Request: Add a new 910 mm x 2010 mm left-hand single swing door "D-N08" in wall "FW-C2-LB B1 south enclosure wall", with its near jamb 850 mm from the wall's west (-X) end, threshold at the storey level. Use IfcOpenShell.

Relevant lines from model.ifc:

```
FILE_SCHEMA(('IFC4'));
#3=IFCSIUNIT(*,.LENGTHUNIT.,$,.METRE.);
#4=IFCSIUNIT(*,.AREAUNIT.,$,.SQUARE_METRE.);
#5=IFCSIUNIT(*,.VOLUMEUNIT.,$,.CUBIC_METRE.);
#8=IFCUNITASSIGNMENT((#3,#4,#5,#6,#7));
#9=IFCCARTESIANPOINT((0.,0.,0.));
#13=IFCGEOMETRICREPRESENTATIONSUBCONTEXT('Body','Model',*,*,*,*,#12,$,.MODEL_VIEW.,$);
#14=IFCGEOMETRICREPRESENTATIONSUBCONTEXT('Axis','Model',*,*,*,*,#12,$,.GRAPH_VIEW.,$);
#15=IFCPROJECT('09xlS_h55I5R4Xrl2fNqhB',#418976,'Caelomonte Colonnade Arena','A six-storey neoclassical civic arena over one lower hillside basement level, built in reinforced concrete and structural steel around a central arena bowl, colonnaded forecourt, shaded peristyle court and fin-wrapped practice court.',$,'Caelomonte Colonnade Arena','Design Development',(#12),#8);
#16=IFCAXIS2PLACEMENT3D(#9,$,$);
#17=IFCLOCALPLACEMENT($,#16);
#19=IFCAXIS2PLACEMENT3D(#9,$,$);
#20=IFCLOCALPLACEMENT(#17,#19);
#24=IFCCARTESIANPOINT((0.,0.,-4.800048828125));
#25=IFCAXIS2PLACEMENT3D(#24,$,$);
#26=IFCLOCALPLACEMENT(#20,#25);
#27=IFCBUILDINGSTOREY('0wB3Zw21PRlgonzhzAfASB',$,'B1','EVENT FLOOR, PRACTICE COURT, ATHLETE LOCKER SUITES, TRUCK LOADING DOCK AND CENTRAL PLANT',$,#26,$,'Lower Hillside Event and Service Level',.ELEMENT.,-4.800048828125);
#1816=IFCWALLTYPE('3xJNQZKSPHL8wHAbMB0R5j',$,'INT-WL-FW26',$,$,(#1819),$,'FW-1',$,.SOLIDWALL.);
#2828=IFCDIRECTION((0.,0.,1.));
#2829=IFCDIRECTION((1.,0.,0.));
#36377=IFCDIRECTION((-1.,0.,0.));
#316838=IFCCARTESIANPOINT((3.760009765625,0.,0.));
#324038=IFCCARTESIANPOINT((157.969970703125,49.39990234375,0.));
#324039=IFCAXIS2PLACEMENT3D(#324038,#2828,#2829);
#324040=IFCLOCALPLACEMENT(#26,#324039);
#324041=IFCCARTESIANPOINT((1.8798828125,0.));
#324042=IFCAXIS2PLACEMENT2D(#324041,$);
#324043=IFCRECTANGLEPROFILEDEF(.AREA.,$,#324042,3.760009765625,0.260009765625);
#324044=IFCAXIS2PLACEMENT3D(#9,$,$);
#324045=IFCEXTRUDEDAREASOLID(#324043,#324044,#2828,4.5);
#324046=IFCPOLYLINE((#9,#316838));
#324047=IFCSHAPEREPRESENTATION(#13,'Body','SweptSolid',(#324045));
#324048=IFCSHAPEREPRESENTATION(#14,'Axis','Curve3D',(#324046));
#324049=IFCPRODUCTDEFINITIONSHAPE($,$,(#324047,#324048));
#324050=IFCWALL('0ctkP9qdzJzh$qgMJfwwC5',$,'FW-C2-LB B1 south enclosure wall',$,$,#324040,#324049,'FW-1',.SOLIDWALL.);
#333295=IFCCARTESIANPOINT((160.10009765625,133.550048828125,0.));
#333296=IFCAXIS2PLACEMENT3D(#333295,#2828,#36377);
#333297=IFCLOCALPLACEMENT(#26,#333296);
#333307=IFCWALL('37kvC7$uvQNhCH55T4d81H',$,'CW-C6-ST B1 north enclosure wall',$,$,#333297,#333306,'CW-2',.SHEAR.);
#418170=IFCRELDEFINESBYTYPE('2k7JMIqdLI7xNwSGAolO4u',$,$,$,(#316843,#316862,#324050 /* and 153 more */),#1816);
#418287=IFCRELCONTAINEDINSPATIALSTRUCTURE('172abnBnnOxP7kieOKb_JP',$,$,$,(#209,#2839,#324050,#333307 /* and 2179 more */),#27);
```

```python
import numpy as np
import ifcopenshell
import ifcopenshell.api.feature
import ifcopenshell.api.geometry
import ifcopenshell.api.root
import ifcopenshell.api.spatial
import ifcopenshell.geom
import ifcopenshell.util.element
import ifcopenshell.util.placement
import ifcopenshell.util.representation
import ifcopenshell.util.shape
import ifcopenshell.util.unit

model = ifcopenshell.open("model.ifc")
unit_scale = ifcopenshell.util.unit.calculate_unit_scale(model)
settings = ifcopenshell.geom.settings()


def volume(element):
    """Net volume in cubic metres, openings subtracted."""
    shape = ifcopenshell.geom.create_shape(settings, element)
    return ifcopenshell.util.shape.get_volume(shape.geometry)


wall = model.by_id(324050)
storey = ifcopenshell.util.element.get_container(wall, ifc_class="IfcBuildingStorey")
context = ifcopenshell.util.representation.get_context(model, "Model", "Body", "MODEL_VIEW")
before = volume(wall)

width, height, from_end, sill = 0.91, 2.01, 0.85, 0.0  # metres

# The wall runs along its own X axis, and the end named is its -X end.
wall_shape = ifcopenshell.geom.create_shape(settings, wall)
x, y, z = ifcopenshell.util.shape.get_vertices(wall_shape.geometry).T
start = x.min() + from_end
face, thickness = float(y.min()), float(y.max() - y.min())
wall_matrix = ifcopenshell.util.placement.get_local_placement(wall.ObjectPlacement)
level = ifcopenshell.util.placement.get_local_placement(storey.ObjectPlacement)[2, 3]


def in_wall(x, y):
    """Placement at x, y metres in the wall's axes, at sill height."""
    matrix = wall_matrix.copy()
    matrix[:, 3] = wall_matrix @ np.array([x / unit_scale, y / unit_scale, 0.0, 1.0])
    matrix[2, 3] = level + sill / unit_scale
    return matrix


# Opening: a box that overshoots both wall faces by 50 mm.
opening = ifcopenshell.api.root.create_entity(model, ifc_class="IfcOpeningElement", predefined_type="OPENING")
box = ifcopenshell.api.geometry.add_wall_representation(
    model, context=context, length=width, height=height, thickness=thickness + 0.1
)
ifcopenshell.api.geometry.assign_representation(model, product=opening, representation=box)
ifcopenshell.api.geometry.edit_object_placement(model, product=opening, matrix=in_wall(start, face - 0.05), is_si=False)
ifcopenshell.api.feature.add_feature(model, feature=opening, element=wall)

door = ifcopenshell.api.root.create_entity(model, ifc_class="IfcDoor", name="D-N08", predefined_type="DOOR")
door.OverallWidth, door.OverallHeight = width / unit_scale, height / unit_scale
door.OperationType = "SINGLE_SWING_LEFT"
body = ifcopenshell.api.geometry.add_door_representation(
    model,
    context=context,
    overall_width=door.OverallWidth,
    overall_height=door.OverallHeight,
    operation_type="SINGLE_SWING_LEFT",
    lining_properties={"LiningDepth": thickness / unit_scale, "ThresholdDepth": thickness / unit_scale},
)
ifcopenshell.api.geometry.assign_representation(model, product=door, representation=body)
ifcopenshell.api.spatial.assign_container(model, products=[door], relating_structure=storey)
ifcopenshell.api.feature.add_filling(model, opening=opening, element=door)

# The lining spans the wall, so the door starts at the wall face.
ifcopenshell.api.geometry.edit_object_placement(model, product=door, matrix=in_wall(start, face), is_si=False)

after = volume(wall)

print(f"wall volume {before:.3f} -> {after:.3f} m3")

model.write("model_v2.ifc")
```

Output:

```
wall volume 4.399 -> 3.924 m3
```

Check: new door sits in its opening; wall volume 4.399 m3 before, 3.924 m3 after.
